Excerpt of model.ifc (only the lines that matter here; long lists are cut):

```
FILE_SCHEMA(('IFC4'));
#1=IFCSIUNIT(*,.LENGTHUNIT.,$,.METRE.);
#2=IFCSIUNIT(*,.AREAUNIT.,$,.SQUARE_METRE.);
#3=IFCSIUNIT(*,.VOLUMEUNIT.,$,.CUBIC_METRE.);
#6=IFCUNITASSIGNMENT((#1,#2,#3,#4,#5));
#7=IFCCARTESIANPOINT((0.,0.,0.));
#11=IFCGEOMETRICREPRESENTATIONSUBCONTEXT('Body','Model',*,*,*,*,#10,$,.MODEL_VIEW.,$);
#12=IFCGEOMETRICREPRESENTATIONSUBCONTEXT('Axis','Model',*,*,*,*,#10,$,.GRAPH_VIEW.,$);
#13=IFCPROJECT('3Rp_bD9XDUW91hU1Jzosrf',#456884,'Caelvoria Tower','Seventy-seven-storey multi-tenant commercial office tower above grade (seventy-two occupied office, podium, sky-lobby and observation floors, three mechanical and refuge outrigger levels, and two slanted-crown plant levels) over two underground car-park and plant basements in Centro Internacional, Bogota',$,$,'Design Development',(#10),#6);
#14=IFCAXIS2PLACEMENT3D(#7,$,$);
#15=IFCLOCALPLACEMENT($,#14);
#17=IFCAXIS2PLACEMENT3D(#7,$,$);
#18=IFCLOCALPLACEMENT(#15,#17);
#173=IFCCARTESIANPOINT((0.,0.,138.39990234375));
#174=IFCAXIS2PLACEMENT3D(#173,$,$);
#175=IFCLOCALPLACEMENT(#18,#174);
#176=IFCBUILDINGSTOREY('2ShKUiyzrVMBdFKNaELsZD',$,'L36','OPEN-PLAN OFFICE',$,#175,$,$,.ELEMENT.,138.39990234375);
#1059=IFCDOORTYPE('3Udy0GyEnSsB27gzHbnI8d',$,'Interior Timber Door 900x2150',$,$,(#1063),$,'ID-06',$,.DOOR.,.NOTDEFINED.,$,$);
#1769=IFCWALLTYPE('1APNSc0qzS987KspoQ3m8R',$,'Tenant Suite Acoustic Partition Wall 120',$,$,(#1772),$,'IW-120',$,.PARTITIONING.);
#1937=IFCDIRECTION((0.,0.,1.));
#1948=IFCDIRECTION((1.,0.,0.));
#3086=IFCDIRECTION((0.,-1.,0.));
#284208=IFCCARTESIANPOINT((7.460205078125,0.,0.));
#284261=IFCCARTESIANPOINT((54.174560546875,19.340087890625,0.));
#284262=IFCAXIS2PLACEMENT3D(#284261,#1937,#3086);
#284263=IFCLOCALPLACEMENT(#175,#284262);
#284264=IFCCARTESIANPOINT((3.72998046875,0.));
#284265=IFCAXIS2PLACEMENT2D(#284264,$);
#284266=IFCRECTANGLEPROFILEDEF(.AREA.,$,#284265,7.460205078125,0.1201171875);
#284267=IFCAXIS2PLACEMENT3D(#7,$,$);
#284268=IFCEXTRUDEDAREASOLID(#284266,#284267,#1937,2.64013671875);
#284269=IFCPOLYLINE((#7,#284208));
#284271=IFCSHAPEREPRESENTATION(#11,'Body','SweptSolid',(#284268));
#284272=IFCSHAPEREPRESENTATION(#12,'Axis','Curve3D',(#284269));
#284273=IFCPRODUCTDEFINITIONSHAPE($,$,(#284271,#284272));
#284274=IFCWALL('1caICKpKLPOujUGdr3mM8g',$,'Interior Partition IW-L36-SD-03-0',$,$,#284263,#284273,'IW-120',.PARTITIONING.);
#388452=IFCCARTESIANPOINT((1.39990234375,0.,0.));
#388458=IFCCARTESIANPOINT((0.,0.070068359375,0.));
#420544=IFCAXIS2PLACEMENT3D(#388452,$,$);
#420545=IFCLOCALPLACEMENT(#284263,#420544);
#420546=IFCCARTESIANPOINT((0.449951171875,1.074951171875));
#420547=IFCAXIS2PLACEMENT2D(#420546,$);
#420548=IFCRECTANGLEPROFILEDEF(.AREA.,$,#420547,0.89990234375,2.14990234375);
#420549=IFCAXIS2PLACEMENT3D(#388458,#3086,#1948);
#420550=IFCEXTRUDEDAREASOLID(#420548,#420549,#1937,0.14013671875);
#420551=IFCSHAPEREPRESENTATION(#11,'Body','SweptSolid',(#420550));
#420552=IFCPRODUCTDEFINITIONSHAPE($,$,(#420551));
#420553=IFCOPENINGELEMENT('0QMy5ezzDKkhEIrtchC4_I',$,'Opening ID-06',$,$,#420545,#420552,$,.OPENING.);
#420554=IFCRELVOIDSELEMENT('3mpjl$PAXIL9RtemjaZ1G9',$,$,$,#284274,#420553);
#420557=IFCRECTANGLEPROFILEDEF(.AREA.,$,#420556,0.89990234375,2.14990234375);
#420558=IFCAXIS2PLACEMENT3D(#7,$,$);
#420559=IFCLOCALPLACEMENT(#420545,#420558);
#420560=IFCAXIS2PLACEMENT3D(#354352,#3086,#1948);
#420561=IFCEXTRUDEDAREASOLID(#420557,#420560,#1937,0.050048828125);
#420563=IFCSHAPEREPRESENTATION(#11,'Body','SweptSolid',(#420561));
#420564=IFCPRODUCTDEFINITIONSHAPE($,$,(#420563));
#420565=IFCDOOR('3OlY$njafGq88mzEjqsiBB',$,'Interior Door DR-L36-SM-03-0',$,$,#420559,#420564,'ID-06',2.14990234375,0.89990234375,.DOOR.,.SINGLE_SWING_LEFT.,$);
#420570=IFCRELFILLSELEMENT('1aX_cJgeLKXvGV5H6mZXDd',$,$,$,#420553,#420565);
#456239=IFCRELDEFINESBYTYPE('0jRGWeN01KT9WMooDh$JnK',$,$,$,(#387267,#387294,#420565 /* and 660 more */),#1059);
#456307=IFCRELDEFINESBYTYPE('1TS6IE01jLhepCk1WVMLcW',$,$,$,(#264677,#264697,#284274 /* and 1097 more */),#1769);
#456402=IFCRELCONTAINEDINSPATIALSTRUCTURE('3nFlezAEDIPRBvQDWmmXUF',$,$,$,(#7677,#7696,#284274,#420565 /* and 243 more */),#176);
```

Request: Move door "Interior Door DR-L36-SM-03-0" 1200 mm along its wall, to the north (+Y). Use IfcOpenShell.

```python
import ifcopenshell
import ifcopenshell.api.geometry
import ifcopenshell.util.placement

model = ifcopenshell.open("model.ifc")

door = model.by_guid("3OlY$njafGq88mzEjqsiBB")
opening = door.FillsVoids[0].RelatingOpeningElement
wall = opening.VoidsElements[0].RelatingBuildingElement

wall_matrix = ifcopenshell.util.placement.get_local_placement(wall.ObjectPlacement)
shift = wall_matrix[:3, 0] * -1.2
before = ifcopenshell.util.placement.get_local_placement(door.ObjectPlacement)[:3, 3].copy()

# The door is placed relative to its opening, so it follows when the opening moves.
matrix = ifcopenshell.util.placement.get_local_placement(opening.ObjectPlacement)
matrix[:3, 3] += shift
ifcopenshell.api.geometry.edit_object_placement(
    model, product=opening, matrix=matrix, is_si=False, should_transform_children=True
)

after = ifcopenshell.util.placement.get_local_placement(door.ObjectPlacement)[:3, 3]
print("door moved by", (after - before).round(3) + 0.0)

model.write("model_rev.ifc")
```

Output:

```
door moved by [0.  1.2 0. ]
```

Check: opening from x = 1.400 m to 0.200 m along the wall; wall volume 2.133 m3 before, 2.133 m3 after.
